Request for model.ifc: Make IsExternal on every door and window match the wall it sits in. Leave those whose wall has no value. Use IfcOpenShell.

First a look at what the model holds.

```python
import ifcopenshell
import ifcopenshell.util.element

model = ifcopenshell.open("model.ifc")
print(model.schema)
seen = {}
for e in model.by_type("IfcDoor") + model.by_type("IfcWindow"):
    if not e.FillsVoids:
        continue
    host = e.FillsVoids[0].RelatingOpeningElement.VoidsElements[0].RelatingBuildingElement
    own = ifcopenshell.util.element.get_pset(e, f"Pset_{e.is_a()[3:].removesuffix('StandardCase')}Common", "IsExternal")
    wall = ifcopenshell.util.element.get_pset(host, "Pset_WallCommon", "IsExternal")
    seen[e.is_a(), own, wall] = seen.get((e.is_a(), own, wall), 0) + 1
for (cls, own, wall), count in sorted(seen.items(), key=str):
    print(count, cls, "IsExternal:", own, "| host wall:", wall)
```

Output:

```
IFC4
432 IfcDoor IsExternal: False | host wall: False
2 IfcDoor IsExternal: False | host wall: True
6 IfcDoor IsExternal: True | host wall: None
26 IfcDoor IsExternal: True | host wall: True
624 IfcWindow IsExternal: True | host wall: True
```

```python
import ifcopenshell
import ifcopenshell.api.pset
import ifcopenshell.util.element

model = ifcopenshell.open("model.ifc")

count = 0
for ifc_class, pset_name in (("IfcDoor", "Pset_DoorCommon"), ("IfcWindow", "Pset_WindowCommon")):
    for e in model.by_type(ifc_class):
        if not e.FillsVoids:
            continue
        host = e.FillsVoids[0].RelatingOpeningElement.VoidsElements[0].RelatingBuildingElement
        external = ifcopenshell.util.element.get_pset(host, "Pset_WallCommon", "IsExternal")
        if external is None or ifcopenshell.util.element.get_pset(e, pset_name, "IsExternal") == external:
            continue
        pset = ifcopenshell.api.pset.add_pset(model, product=e, name=pset_name)
        ifcopenshell.api.pset.edit_pset(model, pset=pset, properties={"IsExternal": external})
        count += 1

print(count, "updated")

model.write("model_edited.ifc")
```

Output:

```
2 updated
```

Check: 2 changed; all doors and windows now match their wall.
